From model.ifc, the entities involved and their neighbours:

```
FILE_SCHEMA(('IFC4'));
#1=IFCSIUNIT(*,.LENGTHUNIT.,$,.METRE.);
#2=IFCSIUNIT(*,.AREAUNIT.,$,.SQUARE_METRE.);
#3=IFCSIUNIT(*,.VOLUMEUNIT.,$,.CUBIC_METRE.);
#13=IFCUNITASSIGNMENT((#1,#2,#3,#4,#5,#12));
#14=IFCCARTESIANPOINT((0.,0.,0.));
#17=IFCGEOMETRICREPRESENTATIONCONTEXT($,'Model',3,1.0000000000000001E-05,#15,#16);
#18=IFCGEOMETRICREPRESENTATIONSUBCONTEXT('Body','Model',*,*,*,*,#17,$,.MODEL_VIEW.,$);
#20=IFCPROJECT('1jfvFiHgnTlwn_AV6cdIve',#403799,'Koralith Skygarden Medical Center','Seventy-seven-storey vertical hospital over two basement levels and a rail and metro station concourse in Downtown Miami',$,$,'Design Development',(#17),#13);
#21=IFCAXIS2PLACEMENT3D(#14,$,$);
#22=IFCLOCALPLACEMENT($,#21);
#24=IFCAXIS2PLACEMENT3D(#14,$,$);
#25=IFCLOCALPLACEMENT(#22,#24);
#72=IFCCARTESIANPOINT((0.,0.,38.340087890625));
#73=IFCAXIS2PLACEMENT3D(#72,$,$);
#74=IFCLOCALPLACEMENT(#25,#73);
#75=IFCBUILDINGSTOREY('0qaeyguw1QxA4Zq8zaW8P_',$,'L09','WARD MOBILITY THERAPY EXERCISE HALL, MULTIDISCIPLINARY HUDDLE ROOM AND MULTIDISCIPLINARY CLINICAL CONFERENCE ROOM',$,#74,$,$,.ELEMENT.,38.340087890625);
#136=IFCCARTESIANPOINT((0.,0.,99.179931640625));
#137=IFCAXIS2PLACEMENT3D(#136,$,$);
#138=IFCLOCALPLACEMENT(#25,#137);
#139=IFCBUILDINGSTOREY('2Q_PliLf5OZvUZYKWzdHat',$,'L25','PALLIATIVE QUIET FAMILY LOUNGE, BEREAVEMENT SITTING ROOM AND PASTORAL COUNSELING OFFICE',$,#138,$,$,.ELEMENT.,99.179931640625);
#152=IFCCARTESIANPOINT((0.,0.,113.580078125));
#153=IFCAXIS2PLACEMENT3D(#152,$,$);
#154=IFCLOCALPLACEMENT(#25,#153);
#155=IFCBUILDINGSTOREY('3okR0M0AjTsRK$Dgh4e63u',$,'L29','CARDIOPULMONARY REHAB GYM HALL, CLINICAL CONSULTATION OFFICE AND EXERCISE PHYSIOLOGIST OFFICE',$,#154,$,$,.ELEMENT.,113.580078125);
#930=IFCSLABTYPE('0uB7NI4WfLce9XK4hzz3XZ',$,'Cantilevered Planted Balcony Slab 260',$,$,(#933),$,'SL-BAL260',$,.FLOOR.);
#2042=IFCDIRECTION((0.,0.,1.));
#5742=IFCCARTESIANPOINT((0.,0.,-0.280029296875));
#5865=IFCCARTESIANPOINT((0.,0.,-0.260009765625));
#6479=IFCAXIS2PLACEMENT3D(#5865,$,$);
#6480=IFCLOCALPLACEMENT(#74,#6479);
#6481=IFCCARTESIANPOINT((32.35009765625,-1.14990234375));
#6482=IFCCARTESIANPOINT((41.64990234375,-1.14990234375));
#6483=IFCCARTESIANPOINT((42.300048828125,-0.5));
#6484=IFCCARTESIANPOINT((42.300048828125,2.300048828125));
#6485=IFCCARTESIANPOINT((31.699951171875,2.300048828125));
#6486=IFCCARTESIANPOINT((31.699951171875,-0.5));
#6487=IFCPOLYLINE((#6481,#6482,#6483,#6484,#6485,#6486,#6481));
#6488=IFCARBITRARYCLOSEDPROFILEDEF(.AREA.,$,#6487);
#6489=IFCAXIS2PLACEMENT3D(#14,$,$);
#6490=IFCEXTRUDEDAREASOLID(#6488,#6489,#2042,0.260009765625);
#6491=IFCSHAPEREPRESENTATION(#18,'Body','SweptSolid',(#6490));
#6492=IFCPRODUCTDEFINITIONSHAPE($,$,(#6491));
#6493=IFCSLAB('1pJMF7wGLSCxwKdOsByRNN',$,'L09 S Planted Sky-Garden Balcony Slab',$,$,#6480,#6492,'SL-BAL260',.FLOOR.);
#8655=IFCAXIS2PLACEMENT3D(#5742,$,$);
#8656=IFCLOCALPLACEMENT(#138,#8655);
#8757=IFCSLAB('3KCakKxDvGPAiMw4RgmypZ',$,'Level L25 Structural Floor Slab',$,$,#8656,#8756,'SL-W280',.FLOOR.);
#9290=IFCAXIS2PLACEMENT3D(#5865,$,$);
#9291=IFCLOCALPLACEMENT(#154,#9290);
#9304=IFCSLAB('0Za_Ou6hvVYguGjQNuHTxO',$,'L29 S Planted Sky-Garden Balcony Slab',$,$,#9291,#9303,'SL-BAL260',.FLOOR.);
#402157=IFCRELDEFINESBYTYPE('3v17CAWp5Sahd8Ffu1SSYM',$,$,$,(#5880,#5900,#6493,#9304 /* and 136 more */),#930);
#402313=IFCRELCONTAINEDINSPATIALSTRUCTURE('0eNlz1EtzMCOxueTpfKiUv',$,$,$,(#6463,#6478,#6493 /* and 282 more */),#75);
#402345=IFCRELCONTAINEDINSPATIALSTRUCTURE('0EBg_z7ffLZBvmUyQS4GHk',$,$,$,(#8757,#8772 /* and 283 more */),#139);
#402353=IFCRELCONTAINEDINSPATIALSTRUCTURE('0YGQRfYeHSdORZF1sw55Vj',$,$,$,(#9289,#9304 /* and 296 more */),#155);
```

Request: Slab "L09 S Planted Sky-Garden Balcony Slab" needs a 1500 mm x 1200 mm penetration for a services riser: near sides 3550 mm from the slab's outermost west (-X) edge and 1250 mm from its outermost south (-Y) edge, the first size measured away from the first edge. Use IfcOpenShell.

```python
import numpy as np
import ifcopenshell
import ifcopenshell.api.feature
import ifcopenshell.api.geometry
import ifcopenshell.api.root
import ifcopenshell.geom
import ifcopenshell.util.placement
import ifcopenshell.util.representation
import ifcopenshell.util.shape
import ifcopenshell.util.unit

model = ifcopenshell.open("model.ifc")
unit_scale = ifcopenshell.util.unit.calculate_unit_scale(model)
settings = ifcopenshell.geom.settings()


def volume(element):
    """Net volume in cubic metres, openings subtracted."""
    shape = ifcopenshell.geom.create_shape(settings, element)
    return ifcopenshell.util.shape.get_volume(shape.geometry)


slab = model.by_id(6493)
before = volume(slab)

# Extent in the slab's own axes, in metres. The edges named are its -X and -Y sides.
slab_shape = ifcopenshell.geom.create_shape(settings, slab)
vertices = ifcopenshell.util.shape.get_vertices(slab_shape.geometry)
x_min, y_min, bottom = vertices.min(axis=0)
top = vertices[:, 2].max()

opening = ifcopenshell.api.root.create_entity(model, ifc_class="IfcOpeningElement", name="Services riser opening", predefined_type="OPENING")
context = ifcopenshell.util.representation.get_context(model, "Model", "Body", "MODEL_VIEW")
width, depth = 1.5, 1.2
outline = [(0.0, 0.0), (width, 0.0), (width, depth), (0.0, depth), (0.0, 0.0)]
# Overshoot both faces by 50 mm so the cut is clean.
shape = ifcopenshell.api.geometry.add_slab_representation(
    model, context=context, depth=top - bottom + 0.1, polyline=outline
)
ifcopenshell.api.geometry.assign_representation(model, product=opening, representation=shape)

matrix = ifcopenshell.util.placement.get_local_placement(slab.ObjectPlacement)
matrix[:, 3] = matrix @ np.append(np.array([x_min + 3.55, y_min + 1.25, bottom - 0.05]) / unit_scale, 1.0)
ifcopenshell.api.geometry.edit_object_placement(model, product=opening, matrix=matrix, is_si=False)
ifcopenshell.api.feature.add_feature(model, feature=opening, element=slab)

after = volume(slab)

print(f"slab volume {before:.3f} -> {after:.3f} m3")

model.write("model-out.ifc")
```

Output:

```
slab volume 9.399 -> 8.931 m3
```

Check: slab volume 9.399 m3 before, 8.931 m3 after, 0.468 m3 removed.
